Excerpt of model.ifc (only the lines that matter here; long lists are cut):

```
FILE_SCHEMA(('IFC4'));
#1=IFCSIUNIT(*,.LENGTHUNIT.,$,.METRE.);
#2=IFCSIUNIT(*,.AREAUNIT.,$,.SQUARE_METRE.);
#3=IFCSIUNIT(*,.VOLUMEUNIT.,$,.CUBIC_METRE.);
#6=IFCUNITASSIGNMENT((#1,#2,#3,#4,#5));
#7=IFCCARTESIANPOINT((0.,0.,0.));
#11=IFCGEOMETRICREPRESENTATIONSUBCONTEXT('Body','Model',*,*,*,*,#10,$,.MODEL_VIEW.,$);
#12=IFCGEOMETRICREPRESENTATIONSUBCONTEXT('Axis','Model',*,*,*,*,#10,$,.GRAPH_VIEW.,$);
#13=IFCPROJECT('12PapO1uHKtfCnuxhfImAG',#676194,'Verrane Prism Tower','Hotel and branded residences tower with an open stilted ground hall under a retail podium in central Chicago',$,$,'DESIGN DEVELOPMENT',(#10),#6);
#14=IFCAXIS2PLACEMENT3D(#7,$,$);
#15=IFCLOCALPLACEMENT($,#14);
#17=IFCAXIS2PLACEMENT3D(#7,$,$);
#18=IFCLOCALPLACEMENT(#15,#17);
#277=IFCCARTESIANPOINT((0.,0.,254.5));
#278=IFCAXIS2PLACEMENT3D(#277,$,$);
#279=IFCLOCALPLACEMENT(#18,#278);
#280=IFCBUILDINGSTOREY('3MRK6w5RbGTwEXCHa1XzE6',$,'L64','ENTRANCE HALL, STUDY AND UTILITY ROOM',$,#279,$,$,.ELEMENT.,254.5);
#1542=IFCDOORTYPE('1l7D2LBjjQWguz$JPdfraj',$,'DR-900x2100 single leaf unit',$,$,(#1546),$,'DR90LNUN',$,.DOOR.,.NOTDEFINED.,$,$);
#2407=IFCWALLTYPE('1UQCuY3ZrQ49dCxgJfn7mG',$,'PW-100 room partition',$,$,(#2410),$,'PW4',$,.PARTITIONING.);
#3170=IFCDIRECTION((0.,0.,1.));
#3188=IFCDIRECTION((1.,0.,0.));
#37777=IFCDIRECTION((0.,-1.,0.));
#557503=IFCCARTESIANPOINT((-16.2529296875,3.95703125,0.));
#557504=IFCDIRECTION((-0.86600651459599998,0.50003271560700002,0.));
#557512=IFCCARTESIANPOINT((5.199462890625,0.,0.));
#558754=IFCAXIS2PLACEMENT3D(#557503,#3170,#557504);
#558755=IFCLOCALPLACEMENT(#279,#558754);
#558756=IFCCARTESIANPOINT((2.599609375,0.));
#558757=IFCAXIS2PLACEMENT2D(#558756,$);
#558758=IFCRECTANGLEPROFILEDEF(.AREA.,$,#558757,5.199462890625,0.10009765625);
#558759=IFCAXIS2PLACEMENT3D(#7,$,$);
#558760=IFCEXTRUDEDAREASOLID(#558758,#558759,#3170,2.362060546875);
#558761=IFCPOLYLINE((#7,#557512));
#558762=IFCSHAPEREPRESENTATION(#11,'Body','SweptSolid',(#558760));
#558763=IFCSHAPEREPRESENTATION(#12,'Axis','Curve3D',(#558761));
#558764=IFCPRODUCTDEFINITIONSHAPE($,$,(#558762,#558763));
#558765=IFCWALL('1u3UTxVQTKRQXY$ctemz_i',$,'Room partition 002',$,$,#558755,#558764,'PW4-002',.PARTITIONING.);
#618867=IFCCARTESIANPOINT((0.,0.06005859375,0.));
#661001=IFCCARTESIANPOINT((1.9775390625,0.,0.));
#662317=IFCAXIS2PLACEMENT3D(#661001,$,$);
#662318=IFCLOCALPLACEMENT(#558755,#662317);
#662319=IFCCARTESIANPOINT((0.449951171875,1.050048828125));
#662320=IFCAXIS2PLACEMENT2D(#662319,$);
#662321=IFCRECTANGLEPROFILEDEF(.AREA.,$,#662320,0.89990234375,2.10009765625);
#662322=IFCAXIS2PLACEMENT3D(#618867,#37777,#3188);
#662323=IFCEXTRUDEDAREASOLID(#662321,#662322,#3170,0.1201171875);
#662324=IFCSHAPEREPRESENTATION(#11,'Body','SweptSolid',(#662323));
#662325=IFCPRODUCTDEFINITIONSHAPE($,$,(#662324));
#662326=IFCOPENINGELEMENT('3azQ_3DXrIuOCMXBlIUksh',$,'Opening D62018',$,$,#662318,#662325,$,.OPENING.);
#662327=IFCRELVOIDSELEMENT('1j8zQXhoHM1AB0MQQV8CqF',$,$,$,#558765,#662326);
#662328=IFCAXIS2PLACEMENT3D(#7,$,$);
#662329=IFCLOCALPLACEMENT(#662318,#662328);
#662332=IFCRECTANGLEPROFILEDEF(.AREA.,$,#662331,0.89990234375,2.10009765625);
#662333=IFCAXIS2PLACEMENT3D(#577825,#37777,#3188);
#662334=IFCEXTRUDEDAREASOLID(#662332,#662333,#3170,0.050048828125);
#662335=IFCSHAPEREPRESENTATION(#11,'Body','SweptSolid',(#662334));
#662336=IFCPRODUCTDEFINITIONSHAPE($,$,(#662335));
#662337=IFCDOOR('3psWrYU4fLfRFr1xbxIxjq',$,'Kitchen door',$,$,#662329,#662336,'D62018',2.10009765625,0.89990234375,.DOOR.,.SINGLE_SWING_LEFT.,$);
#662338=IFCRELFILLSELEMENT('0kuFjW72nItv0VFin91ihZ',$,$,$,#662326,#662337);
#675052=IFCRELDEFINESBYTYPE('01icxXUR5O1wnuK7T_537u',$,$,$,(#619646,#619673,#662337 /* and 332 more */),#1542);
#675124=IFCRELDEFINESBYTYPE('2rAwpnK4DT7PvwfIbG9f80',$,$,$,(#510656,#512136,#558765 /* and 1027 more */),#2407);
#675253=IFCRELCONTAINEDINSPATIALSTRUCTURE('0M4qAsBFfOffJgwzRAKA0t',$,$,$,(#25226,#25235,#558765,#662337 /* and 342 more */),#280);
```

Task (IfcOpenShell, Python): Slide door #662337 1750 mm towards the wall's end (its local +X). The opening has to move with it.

```python
import ifcopenshell
import ifcopenshell.api.geometry
import ifcopenshell.util.placement

model = ifcopenshell.open("model.ifc")

door = model.by_id(662337)
opening = door.FillsVoids[0].RelatingOpeningElement
wall = opening.VoidsElements[0].RelatingBuildingElement

wall_matrix = ifcopenshell.util.placement.get_local_placement(wall.ObjectPlacement)
shift = wall_matrix[:3, 0] * 1.75
before = ifcopenshell.util.placement.get_local_placement(door.ObjectPlacement)[:3, 3].copy()

# The door is placed relative to its opening, so it follows when the opening moves.
matrix = ifcopenshell.util.placement.get_local_placement(opening.ObjectPlacement)
matrix[:3, 3] += shift
ifcopenshell.api.geometry.edit_object_placement(
    model, product=opening, matrix=matrix, is_si=False, should_transform_children=True
)

after = ifcopenshell.util.placement.get_local_placement(door.ObjectPlacement)[:3, 3]
print("door moved by", (after - before).round(3) + 0.0)

model.write("model_updated.ifc")
```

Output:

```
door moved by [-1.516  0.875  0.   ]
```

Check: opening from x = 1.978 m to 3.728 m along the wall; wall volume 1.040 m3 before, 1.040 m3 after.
